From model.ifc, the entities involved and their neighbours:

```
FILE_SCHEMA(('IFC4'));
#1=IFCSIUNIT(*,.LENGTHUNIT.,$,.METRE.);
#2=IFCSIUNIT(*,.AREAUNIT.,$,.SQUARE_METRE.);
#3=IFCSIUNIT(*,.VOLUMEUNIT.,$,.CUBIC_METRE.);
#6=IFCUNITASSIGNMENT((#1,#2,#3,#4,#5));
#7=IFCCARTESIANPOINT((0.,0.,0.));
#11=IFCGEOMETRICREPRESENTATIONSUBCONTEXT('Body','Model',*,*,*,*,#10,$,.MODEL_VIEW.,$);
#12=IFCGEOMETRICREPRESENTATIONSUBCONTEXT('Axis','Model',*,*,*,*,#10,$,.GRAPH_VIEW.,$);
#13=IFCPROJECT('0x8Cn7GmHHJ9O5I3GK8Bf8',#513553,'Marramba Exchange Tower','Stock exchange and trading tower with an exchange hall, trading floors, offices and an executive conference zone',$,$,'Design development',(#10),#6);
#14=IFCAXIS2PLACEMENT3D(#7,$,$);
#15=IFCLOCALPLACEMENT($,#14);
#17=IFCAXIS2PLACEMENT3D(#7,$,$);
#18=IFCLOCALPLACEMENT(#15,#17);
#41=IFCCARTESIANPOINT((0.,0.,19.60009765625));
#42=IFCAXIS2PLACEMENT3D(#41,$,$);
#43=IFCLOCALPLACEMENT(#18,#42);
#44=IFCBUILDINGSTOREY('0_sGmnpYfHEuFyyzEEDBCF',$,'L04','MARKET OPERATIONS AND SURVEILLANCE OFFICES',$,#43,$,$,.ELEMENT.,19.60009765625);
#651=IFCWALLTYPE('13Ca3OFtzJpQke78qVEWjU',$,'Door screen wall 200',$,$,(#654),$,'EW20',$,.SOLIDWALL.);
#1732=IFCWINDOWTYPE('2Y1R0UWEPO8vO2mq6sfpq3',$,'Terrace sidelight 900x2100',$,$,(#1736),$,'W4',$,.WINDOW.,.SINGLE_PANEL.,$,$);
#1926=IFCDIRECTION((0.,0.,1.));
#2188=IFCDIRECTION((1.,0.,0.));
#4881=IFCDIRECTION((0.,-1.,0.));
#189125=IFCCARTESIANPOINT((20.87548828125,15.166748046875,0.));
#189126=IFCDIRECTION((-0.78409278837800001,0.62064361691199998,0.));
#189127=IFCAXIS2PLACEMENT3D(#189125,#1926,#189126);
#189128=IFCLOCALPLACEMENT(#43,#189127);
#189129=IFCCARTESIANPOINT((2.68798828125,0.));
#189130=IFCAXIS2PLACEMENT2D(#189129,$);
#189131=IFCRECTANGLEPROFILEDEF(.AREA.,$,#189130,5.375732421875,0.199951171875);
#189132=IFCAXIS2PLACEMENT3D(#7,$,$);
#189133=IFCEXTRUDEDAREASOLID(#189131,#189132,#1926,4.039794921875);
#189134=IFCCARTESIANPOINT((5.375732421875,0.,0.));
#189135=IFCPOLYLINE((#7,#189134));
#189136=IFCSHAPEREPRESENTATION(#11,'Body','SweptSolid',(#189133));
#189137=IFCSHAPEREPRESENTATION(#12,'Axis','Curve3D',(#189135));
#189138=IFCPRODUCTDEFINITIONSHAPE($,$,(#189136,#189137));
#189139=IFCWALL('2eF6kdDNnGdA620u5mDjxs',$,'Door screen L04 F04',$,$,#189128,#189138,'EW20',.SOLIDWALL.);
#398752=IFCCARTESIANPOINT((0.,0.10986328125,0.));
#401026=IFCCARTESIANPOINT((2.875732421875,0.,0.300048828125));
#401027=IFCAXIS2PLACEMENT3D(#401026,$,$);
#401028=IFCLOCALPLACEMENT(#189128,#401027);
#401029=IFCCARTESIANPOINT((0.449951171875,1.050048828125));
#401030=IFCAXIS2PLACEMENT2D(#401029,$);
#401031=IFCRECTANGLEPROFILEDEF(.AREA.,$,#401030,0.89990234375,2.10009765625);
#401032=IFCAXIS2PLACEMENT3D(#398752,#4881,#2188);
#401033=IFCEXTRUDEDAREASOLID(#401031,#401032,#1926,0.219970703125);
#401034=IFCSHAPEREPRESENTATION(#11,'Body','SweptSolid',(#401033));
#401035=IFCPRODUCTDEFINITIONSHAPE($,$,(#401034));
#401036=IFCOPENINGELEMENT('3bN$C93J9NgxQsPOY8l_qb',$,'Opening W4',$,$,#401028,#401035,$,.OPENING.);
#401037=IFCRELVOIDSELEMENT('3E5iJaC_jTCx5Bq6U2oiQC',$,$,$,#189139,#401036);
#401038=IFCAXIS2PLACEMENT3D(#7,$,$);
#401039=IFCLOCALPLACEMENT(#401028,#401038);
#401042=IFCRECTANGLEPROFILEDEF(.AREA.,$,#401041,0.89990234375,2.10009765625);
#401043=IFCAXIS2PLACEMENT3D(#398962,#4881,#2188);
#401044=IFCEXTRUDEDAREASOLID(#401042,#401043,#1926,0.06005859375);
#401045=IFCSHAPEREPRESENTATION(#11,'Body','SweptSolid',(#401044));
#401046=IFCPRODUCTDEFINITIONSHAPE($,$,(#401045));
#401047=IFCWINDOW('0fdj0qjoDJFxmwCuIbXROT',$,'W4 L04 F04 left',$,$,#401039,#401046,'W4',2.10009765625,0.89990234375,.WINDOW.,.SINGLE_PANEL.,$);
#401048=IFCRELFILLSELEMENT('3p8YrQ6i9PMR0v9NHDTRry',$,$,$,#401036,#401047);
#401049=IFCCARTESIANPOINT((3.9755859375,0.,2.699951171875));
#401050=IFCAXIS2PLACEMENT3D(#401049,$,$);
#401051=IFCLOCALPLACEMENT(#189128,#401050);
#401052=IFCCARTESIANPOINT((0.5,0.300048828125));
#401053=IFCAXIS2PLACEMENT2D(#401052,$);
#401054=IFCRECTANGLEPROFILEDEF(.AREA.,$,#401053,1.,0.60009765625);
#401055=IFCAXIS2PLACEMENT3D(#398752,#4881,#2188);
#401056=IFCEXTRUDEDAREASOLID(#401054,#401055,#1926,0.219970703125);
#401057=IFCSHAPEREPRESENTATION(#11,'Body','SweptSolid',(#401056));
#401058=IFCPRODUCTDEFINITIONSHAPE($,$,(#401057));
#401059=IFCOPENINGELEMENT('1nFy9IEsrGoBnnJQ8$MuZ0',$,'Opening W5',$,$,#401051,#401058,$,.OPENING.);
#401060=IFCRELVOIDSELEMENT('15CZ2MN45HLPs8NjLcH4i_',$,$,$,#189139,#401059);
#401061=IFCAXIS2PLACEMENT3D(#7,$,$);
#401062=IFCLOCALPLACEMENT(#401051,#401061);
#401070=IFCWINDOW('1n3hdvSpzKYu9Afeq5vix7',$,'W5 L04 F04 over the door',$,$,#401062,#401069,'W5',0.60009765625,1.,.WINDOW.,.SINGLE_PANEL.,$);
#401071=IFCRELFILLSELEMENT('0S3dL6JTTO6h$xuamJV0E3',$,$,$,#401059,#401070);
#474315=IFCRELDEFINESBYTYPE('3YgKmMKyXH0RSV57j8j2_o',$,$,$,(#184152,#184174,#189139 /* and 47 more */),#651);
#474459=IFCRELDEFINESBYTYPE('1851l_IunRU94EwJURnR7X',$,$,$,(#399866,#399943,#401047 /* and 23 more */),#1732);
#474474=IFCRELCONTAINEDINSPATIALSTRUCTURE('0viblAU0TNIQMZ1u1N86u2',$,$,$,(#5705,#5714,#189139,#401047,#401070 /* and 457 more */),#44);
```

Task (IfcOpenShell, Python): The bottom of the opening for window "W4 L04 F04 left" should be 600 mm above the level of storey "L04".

```python
import numpy as np
import ifcopenshell
import ifcopenshell.api.geometry
import ifcopenshell.geom
import ifcopenshell.util.element
import ifcopenshell.util.placement
import ifcopenshell.util.shape
import ifcopenshell.util.unit

model = ifcopenshell.open("model.ifc")
unit_scale = ifcopenshell.util.unit.calculate_unit_scale(model)

window = model.by_guid("0fdj0qjoDJFxmwCuIbXROT")
opening = window.FillsVoids[0].RelatingOpeningElement
storey = ifcopenshell.util.element.get_container(window, ifc_class="IfcBuildingStorey")
level = ifcopenshell.util.placement.get_local_placement(storey.ObjectPlacement)[2, 3]

# The opening's origin need not be at the sill, so measure its lowest point.
shape = ifcopenshell.geom.create_shape(ifcopenshell.geom.settings(), opening)
bottom = ifcopenshell.util.shape.get_shape_bottom_elevation(shape, shape.geometry) / unit_scale
dz = level + 0.6 / unit_scale - bottom

shift = np.array([0.0, 0.0, dz])
# The window is placed relative to its opening, so it follows when the opening moves.
matrix = ifcopenshell.util.placement.get_local_placement(opening.ObjectPlacement)
matrix[:3, 3] += shift
ifcopenshell.api.geometry.edit_object_placement(
    model, product=opening, matrix=matrix, is_si=False, should_transform_children=True
)

print(f"moved by {dz * unit_scale:+.3f} m")

model.write("model_v2.ifc")
```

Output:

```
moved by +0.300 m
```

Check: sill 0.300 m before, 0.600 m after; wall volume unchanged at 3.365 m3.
